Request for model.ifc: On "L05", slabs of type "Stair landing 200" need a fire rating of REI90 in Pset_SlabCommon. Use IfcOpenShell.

First a look at what the model holds.

```python
import ifcopenshell
import ifcopenshell.util.element

model = ifcopenshell.open("model.ifc")
print(model.schema)
storey = next(s for s in model.by_type("IfcBuildingStorey") if s.Name == "L05")
slabs = [e for e in ifcopenshell.util.element.get_decomposition(storey) if e.is_a("IfcSlab")]
seen = {}
for e in slabs:
    element_type = ifcopenshell.util.element.get_type(e)
    key = (element_type.Name if element_type != e and element_type else None, ifcopenshell.util.element.get_pset(e, "Pset_SlabCommon", "FireRating"))
    seen[key] = seen.get(key, 0) + 1
for (name, value), count in sorted(seen.items(), key=str):
    print(count, "x", name, "|", value)
```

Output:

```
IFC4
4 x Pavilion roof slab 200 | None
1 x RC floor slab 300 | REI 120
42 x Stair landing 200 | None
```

```python
import ifcopenshell
import ifcopenshell.api.pset
import ifcopenshell.util.element

model = ifcopenshell.open("model.ifc")

storey = next(s for s in model.by_type("IfcBuildingStorey") if s.Name == "L05")
slabs = [e for e in ifcopenshell.util.element.get_decomposition(storey) if e.is_a("IfcSlab")]

count = 0
for e in slabs:
    element_type = ifcopenshell.util.element.get_type(e)
    if element_type in (None, e) or element_type.Name != "Stair landing 200":
        continue
    # add_pset returns the element's existing set when there is one.
    pset = ifcopenshell.api.pset.add_pset(model, product=e, name="Pset_SlabCommon")
    ifcopenshell.api.pset.edit_pset(model, pset=pset, properties={"FireRating": "REI90"})
    count += 1

print(count, "slabs updated")

model.write("model_v2.ifc")
```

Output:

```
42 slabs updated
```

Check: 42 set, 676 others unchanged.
